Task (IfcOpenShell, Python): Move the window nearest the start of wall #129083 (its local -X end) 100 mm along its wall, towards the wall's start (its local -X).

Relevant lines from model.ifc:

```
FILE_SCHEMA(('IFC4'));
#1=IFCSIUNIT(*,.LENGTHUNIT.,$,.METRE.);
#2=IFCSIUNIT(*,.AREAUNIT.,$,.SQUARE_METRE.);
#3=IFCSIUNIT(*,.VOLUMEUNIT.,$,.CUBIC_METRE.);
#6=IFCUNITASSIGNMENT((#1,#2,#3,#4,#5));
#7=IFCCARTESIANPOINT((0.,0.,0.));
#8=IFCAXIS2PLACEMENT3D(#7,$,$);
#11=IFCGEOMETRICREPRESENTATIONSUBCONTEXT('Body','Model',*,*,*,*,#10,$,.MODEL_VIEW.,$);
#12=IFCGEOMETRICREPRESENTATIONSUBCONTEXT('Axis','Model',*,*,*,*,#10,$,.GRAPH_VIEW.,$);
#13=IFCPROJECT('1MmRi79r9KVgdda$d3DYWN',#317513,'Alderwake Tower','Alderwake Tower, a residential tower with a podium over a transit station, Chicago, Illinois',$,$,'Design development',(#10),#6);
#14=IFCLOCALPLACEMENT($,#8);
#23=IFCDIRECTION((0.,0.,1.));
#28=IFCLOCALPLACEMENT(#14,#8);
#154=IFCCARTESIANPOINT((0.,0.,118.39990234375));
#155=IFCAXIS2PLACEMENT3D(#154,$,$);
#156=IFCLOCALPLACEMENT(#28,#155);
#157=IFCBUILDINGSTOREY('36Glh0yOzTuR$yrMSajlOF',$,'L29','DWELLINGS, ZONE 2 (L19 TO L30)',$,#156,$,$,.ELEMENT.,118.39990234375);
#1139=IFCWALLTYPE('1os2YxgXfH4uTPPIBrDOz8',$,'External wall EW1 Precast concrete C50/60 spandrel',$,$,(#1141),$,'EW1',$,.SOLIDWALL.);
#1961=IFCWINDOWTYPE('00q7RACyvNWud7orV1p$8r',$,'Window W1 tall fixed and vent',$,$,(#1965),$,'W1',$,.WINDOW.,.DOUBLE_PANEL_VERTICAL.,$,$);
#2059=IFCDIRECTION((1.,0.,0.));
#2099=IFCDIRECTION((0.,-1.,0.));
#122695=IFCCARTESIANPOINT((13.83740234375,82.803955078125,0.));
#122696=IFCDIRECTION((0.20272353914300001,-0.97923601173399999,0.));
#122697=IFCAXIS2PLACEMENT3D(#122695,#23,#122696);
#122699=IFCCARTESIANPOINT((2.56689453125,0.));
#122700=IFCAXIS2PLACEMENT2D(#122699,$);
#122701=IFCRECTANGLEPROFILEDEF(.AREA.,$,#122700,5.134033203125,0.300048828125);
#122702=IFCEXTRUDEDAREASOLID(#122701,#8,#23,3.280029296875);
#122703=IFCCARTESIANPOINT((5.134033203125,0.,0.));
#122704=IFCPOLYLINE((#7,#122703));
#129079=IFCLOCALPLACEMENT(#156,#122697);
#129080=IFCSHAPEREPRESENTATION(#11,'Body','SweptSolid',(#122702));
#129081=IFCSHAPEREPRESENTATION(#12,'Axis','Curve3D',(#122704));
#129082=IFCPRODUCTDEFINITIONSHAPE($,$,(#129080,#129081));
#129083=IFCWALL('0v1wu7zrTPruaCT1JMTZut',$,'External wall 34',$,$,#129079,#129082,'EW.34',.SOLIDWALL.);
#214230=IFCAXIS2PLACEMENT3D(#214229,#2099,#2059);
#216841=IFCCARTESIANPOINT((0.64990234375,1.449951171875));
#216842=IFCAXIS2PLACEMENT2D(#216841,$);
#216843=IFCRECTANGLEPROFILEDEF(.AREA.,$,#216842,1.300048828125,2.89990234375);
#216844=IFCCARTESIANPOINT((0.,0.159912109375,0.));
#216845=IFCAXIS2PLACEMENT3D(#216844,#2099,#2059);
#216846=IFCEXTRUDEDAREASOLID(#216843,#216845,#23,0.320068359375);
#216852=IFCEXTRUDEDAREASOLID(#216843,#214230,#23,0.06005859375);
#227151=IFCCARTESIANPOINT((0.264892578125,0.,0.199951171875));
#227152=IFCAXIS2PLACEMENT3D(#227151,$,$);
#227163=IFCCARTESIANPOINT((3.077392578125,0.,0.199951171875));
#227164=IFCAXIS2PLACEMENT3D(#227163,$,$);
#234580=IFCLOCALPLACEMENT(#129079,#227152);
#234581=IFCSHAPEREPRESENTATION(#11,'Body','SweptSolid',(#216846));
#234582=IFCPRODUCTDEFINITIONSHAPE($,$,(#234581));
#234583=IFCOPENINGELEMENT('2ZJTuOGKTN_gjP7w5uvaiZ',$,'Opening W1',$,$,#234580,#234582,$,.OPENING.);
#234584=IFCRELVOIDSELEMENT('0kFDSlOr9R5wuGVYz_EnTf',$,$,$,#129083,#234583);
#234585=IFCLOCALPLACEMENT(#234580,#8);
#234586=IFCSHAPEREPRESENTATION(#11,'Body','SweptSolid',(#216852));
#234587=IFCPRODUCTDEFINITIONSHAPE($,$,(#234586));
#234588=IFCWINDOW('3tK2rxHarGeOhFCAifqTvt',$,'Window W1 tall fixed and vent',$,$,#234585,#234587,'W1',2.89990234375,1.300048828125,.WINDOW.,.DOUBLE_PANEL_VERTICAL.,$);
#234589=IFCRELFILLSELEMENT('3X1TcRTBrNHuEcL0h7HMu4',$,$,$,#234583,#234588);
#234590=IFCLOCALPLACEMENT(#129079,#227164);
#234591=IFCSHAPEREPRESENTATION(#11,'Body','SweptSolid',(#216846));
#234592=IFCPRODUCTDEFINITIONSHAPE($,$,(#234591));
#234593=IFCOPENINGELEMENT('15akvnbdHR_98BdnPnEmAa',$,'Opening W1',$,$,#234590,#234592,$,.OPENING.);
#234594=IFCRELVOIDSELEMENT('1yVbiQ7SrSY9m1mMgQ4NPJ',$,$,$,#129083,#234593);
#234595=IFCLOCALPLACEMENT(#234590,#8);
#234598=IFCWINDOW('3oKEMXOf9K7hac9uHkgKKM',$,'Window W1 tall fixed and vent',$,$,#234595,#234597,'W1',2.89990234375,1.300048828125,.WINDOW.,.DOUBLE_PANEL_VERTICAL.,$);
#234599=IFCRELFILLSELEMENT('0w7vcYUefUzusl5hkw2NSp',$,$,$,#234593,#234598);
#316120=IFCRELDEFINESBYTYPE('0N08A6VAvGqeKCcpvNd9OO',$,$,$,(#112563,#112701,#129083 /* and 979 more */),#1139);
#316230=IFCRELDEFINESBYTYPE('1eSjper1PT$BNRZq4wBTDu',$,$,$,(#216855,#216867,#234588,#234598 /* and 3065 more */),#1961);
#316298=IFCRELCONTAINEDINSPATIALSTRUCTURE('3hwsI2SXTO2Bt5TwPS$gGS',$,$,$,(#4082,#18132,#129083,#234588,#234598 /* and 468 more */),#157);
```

```python
import ifcopenshell
import ifcopenshell.api.geometry
import ifcopenshell.util.placement
import ifcopenshell.util.unit

model = ifcopenshell.open("model.ifc")
unit_scale = ifcopenshell.util.unit.calculate_unit_scale(model)

window = model.by_id(234588)
opening = window.FillsVoids[0].RelatingOpeningElement
wall = opening.VoidsElements[0].RelatingBuildingElement

wall_matrix = ifcopenshell.util.placement.get_local_placement(wall.ObjectPlacement)
shift = wall_matrix[:3, 0] * -0.1 / unit_scale
before = ifcopenshell.util.placement.get_local_placement(window.ObjectPlacement)[:3, 3].copy()

# The window is placed relative to its opening, so it follows when the opening moves.
matrix = ifcopenshell.util.placement.get_local_placement(opening.ObjectPlacement)
matrix[:3, 3] += shift
ifcopenshell.api.geometry.edit_object_placement(
    model, product=opening, matrix=matrix, is_si=False, should_transform_children=True
)

after = ifcopenshell.util.placement.get_local_placement(window.ObjectPlacement)[:3, 3]
print("window moved by", (after - before).round(3) + 0.0)

model.write("model_edited.ifc")
```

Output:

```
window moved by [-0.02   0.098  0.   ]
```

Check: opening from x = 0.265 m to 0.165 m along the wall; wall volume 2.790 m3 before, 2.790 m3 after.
